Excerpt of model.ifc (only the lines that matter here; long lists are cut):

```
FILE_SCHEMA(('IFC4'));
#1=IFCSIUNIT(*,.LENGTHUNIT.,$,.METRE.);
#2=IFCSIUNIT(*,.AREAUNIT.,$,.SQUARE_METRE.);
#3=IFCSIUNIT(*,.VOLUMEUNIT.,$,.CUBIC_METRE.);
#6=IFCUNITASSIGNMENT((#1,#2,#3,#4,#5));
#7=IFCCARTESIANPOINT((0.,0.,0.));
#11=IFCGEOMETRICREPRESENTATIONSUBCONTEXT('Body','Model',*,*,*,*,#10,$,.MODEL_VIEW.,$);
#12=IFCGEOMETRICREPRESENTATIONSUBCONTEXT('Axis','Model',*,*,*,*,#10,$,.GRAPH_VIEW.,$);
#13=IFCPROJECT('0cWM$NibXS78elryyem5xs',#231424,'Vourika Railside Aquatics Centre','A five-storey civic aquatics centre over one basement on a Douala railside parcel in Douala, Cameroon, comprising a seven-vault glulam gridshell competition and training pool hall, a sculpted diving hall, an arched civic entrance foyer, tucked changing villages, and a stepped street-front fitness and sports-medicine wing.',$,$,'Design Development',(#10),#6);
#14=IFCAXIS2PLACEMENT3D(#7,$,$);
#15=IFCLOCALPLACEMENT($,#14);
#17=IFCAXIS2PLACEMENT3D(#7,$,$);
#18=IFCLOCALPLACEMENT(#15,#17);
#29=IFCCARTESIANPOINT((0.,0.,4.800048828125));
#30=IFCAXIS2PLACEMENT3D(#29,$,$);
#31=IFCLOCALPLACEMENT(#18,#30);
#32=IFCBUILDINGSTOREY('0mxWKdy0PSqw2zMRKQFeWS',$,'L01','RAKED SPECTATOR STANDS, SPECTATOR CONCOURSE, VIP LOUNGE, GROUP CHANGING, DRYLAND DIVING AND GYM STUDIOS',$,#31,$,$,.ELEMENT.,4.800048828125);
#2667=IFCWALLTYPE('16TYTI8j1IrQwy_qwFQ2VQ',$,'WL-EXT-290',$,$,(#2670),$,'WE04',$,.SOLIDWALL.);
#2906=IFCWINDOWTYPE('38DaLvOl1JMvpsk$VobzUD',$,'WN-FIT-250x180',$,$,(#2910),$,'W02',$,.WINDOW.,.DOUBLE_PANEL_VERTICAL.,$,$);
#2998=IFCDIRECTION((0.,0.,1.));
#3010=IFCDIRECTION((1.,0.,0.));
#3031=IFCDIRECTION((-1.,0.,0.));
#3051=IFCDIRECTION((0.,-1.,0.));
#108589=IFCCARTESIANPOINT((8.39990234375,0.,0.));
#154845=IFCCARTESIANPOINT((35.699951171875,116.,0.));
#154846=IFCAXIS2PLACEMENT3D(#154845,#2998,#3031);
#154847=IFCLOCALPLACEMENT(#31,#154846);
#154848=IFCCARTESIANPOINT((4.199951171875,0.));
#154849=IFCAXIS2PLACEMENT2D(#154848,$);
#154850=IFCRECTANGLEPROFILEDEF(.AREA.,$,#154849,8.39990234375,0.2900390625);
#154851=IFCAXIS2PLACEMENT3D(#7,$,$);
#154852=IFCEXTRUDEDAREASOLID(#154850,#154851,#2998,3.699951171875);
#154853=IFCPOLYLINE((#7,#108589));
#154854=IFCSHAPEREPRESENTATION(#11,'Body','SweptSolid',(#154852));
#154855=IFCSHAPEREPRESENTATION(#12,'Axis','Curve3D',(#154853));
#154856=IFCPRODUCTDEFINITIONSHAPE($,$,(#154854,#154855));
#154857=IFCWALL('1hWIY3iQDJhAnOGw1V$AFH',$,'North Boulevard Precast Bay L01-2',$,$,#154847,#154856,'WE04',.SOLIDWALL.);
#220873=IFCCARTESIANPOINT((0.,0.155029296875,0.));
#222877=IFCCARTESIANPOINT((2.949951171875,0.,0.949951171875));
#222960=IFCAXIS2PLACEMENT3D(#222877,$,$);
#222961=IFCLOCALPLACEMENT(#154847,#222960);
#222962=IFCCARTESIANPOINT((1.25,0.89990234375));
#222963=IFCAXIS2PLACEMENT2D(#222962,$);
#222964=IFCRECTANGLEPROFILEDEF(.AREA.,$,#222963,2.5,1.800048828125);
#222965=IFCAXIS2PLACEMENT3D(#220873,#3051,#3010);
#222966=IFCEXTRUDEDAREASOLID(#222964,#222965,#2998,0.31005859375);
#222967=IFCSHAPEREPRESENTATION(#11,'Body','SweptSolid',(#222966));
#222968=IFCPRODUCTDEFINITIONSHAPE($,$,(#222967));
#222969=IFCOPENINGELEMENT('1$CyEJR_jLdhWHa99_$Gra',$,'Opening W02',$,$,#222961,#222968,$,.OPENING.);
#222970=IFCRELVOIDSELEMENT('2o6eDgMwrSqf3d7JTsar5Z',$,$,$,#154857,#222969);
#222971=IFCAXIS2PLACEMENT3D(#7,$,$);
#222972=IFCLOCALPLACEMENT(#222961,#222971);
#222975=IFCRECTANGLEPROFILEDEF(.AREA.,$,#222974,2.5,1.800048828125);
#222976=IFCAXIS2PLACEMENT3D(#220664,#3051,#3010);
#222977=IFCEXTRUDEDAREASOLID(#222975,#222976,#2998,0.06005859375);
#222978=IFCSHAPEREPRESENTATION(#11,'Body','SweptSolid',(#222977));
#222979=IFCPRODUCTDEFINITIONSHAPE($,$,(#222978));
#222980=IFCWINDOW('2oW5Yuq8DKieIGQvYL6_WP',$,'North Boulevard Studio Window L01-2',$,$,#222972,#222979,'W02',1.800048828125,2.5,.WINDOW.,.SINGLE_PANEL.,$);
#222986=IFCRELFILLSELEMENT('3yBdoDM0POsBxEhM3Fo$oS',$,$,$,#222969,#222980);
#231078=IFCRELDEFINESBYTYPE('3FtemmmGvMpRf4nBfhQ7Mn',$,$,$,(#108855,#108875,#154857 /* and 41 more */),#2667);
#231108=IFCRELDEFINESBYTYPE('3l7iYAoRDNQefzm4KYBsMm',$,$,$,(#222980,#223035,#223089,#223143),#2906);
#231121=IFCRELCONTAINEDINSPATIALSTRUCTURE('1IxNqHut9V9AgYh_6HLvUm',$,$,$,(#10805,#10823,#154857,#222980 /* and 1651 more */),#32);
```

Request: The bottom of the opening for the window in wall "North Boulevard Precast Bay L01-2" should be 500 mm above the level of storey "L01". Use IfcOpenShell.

```python
import numpy as np
import ifcopenshell
import ifcopenshell.api.geometry
import ifcopenshell.geom
import ifcopenshell.util.element
import ifcopenshell.util.placement
import ifcopenshell.util.shape
import ifcopenshell.util.unit

model = ifcopenshell.open("model.ifc")
unit_scale = ifcopenshell.util.unit.calculate_unit_scale(model)

window = model.by_guid("2oW5Yuq8DKieIGQvYL6_WP")
opening = window.FillsVoids[0].RelatingOpeningElement
storey = ifcopenshell.util.element.get_container(window, ifc_class="IfcBuildingStorey")
level = ifcopenshell.util.placement.get_local_placement(storey.ObjectPlacement)[2, 3]

# The opening's origin need not be at the sill, so measure its lowest point.
shape = ifcopenshell.geom.create_shape(ifcopenshell.geom.settings(), opening)
bottom = ifcopenshell.util.shape.get_shape_bottom_elevation(shape, shape.geometry) / unit_scale
dz = level + 0.5 / unit_scale - bottom

shift = np.array([0.0, 0.0, dz])
# The window is placed relative to its opening, so it follows when the opening moves.
matrix = ifcopenshell.util.placement.get_local_placement(opening.ObjectPlacement)
matrix[:3, 3] += shift
ifcopenshell.api.geometry.edit_object_placement(
    model, product=opening, matrix=matrix, is_si=False, should_transform_children=True
)

print(f"moved by {dz * unit_scale:+.3f} m")

model.write("model_edited.ifc")
```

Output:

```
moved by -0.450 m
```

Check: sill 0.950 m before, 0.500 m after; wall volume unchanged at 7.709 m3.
